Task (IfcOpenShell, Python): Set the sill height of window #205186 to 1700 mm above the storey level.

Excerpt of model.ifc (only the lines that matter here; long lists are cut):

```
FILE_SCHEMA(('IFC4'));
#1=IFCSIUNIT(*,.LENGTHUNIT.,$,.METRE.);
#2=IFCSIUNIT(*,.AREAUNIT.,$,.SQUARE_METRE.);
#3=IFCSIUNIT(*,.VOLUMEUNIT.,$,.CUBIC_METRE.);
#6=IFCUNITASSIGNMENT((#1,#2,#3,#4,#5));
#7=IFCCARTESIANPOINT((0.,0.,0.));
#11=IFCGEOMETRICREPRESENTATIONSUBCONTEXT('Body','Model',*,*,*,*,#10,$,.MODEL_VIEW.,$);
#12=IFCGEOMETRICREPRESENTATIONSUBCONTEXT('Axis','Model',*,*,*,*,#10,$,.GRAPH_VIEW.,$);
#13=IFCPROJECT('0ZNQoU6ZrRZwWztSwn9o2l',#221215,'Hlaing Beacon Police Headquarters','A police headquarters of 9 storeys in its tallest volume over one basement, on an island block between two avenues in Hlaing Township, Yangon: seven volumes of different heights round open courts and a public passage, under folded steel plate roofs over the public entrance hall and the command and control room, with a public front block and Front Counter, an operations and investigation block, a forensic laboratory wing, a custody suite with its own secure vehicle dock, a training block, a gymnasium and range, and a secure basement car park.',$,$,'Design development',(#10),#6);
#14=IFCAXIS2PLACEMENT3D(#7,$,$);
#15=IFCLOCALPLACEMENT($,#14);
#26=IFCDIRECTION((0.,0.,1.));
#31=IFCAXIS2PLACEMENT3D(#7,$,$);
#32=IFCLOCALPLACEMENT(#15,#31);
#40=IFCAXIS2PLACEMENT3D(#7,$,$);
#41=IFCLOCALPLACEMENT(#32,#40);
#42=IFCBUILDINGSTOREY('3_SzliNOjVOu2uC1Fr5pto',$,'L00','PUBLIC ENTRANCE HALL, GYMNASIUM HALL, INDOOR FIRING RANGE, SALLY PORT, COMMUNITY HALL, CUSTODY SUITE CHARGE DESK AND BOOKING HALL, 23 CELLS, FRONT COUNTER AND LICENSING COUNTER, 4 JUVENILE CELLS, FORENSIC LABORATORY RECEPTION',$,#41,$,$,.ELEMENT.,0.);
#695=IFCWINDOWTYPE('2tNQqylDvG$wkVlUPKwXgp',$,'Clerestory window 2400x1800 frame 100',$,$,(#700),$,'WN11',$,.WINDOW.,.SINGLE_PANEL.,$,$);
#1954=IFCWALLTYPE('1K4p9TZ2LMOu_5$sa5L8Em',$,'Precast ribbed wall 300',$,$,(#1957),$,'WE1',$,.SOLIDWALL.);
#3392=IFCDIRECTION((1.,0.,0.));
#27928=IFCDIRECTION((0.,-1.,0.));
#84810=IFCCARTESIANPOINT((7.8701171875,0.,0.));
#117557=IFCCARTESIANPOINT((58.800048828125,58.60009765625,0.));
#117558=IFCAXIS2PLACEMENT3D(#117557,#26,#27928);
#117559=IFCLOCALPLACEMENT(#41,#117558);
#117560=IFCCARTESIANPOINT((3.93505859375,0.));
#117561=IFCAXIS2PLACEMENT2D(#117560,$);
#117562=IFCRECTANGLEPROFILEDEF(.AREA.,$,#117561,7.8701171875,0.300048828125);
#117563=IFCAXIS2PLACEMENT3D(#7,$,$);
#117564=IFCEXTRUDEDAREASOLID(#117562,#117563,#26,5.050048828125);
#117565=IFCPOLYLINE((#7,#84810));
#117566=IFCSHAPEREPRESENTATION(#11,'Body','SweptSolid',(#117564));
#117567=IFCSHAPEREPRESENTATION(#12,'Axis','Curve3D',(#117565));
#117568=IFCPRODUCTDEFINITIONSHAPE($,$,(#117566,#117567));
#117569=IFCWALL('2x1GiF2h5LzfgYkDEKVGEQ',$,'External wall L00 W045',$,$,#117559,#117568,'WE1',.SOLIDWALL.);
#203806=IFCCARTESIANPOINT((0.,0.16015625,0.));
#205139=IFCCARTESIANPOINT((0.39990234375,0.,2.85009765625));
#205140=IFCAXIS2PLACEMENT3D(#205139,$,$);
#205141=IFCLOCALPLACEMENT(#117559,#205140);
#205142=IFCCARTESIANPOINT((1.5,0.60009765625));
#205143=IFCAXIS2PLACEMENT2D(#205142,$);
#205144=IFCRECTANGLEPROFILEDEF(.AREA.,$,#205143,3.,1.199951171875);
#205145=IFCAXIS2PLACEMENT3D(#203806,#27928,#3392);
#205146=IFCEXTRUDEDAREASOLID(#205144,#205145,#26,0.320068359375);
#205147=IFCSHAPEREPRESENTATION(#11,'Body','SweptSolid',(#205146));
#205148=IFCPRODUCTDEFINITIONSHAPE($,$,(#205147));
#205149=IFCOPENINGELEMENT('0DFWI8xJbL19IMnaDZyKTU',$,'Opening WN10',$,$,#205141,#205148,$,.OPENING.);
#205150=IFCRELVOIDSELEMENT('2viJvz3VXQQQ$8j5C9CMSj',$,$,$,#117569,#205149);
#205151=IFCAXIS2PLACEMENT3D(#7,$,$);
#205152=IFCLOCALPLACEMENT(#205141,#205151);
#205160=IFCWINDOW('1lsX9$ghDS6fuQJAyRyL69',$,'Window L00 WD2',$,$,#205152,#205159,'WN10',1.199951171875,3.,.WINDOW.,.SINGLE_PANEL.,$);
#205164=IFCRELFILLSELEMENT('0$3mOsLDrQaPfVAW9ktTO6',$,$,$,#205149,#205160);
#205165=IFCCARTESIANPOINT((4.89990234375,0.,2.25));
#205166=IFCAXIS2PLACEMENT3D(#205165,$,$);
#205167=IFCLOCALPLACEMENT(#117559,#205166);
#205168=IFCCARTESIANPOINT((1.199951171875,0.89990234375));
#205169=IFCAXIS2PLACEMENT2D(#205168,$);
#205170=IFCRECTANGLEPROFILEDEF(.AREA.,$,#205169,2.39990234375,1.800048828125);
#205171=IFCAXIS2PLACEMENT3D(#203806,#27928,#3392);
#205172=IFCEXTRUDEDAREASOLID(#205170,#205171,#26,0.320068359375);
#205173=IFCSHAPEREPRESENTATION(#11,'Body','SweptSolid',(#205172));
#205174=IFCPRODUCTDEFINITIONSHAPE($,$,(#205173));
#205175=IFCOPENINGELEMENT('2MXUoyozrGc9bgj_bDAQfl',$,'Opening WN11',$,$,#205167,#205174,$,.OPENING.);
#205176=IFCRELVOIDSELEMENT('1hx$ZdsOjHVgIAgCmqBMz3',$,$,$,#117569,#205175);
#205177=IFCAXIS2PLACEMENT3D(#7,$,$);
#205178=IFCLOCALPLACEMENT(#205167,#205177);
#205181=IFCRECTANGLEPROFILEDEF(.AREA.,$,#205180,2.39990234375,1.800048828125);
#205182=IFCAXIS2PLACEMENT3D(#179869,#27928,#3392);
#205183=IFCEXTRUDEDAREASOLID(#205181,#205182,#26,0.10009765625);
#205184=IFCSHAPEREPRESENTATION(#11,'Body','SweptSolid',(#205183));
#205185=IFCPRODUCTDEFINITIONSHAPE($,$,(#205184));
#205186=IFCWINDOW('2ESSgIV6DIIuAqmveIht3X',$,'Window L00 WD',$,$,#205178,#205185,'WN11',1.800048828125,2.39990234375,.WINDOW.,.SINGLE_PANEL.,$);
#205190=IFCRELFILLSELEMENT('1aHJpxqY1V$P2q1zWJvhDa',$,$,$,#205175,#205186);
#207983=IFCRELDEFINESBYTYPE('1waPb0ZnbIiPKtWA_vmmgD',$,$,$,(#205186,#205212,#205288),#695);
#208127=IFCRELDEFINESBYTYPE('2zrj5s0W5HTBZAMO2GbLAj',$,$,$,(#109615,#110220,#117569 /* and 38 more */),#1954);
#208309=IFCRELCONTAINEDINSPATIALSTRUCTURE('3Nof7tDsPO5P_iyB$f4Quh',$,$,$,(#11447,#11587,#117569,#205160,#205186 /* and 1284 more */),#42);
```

```python
import numpy as np
import ifcopenshell
import ifcopenshell.api.geometry
import ifcopenshell.geom
import ifcopenshell.util.element
import ifcopenshell.util.placement
import ifcopenshell.util.shape
import ifcopenshell.util.unit

model = ifcopenshell.open("model.ifc")
unit_scale = ifcopenshell.util.unit.calculate_unit_scale(model)

window = model.by_id(205186)
opening = window.FillsVoids[0].RelatingOpeningElement
storey = ifcopenshell.util.element.get_container(window, ifc_class="IfcBuildingStorey")
level = ifcopenshell.util.placement.get_local_placement(storey.ObjectPlacement)[2, 3]

# The opening's origin need not be at the sill, so measure its lowest point.
shape = ifcopenshell.geom.create_shape(ifcopenshell.geom.settings(), opening)
bottom = ifcopenshell.util.shape.get_shape_bottom_elevation(shape, shape.geometry) / unit_scale
dz = level + 1.7 - bottom

shift = np.array([0.0, 0.0, dz])
# The window is placed relative to its opening, so it follows when the opening moves.
matrix = ifcopenshell.util.placement.get_local_placement(opening.ObjectPlacement)
matrix[:3, 3] += shift
ifcopenshell.api.geometry.edit_object_placement(
    model, product=opening, matrix=matrix, is_si=False, should_transform_children=True
)

print(f"moved by {dz * unit_scale:+.3f} m")

model.write("model_rev.ifc")
```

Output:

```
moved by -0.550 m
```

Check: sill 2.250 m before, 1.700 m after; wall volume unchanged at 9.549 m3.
